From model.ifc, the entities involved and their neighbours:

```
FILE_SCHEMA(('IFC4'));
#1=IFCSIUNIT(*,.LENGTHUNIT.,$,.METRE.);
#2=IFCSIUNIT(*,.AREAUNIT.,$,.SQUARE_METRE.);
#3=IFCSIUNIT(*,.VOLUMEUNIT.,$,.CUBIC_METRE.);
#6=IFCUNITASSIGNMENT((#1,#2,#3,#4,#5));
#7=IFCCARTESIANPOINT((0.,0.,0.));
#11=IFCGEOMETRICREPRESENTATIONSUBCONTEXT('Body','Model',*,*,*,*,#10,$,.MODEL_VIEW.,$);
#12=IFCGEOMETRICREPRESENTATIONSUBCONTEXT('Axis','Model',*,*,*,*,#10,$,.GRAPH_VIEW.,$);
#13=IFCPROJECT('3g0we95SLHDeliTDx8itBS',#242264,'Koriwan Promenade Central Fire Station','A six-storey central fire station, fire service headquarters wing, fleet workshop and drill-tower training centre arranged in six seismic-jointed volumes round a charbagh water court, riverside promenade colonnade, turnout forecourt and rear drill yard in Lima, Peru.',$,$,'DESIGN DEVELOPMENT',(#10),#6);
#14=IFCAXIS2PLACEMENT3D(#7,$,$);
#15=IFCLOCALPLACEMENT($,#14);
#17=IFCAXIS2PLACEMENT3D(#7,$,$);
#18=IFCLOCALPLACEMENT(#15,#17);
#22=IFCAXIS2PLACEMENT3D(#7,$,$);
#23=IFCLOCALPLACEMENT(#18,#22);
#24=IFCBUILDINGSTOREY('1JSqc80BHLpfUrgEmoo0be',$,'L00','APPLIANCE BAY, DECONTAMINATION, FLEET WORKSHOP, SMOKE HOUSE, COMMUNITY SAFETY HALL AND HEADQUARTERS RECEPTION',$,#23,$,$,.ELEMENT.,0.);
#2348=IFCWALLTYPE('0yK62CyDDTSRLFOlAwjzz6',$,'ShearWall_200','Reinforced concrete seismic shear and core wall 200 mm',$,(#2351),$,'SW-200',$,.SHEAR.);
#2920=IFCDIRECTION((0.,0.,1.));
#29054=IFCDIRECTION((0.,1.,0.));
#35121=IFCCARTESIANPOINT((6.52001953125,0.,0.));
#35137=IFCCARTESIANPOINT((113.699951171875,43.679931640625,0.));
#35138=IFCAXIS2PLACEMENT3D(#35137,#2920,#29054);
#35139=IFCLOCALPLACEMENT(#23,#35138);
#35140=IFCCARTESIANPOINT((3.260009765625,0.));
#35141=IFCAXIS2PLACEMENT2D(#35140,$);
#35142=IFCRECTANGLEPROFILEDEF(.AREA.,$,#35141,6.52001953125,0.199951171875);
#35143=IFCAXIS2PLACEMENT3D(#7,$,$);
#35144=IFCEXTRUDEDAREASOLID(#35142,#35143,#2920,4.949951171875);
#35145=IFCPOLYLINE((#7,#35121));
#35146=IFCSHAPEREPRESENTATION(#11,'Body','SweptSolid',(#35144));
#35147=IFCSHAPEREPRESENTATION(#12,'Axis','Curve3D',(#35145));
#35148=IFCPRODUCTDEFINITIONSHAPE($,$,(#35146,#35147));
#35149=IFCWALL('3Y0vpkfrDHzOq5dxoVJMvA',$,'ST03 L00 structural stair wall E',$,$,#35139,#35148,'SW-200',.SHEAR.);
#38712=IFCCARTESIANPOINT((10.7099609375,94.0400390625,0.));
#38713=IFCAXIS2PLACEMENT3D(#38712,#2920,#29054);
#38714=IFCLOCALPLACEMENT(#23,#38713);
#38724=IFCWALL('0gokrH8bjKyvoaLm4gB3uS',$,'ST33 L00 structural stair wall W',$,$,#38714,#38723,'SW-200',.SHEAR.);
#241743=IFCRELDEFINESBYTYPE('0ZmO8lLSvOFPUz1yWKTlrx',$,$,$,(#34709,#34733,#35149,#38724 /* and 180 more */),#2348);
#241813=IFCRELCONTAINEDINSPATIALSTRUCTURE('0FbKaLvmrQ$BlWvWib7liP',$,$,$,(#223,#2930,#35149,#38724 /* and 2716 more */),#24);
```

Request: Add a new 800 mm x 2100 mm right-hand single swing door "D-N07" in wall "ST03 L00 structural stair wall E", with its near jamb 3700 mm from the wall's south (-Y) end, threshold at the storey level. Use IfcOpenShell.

```python
import numpy as np
import ifcopenshell
import ifcopenshell.api.feature
import ifcopenshell.api.geometry
import ifcopenshell.api.root
import ifcopenshell.api.spatial
import ifcopenshell.geom
import ifcopenshell.util.element
import ifcopenshell.util.placement
import ifcopenshell.util.representation
import ifcopenshell.util.shape
import ifcopenshell.util.unit

model = ifcopenshell.open("model.ifc")
unit_scale = ifcopenshell.util.unit.calculate_unit_scale(model)
settings = ifcopenshell.geom.settings()


def volume(element):
    """Net volume in cubic metres, openings subtracted."""
    shape = ifcopenshell.geom.create_shape(settings, element)
    return ifcopenshell.util.shape.get_volume(shape.geometry)


wall = model.by_guid("3Y0vpkfrDHzOq5dxoVJMvA")
storey = ifcopenshell.util.element.get_container(wall, ifc_class="IfcBuildingStorey")
context = ifcopenshell.util.representation.get_context(model, "Model", "Body", "MODEL_VIEW")
before = volume(wall)

width, height, from_end, sill = 0.8, 2.1, 3.7, 0.0  # metres

# The wall runs along its own X axis, and the end named is its -X end.
wall_shape = ifcopenshell.geom.create_shape(settings, wall)
x, y, z = ifcopenshell.util.shape.get_vertices(wall_shape.geometry).T
start = x.min() + from_end
face, thickness = float(y.min()), float(y.max() - y.min())
wall_matrix = ifcopenshell.util.placement.get_local_placement(wall.ObjectPlacement)
level = ifcopenshell.util.placement.get_local_placement(storey.ObjectPlacement)[2, 3]


def in_wall(x, y):
    """Placement at x, y metres in the wall's axes, at sill height."""
    matrix = wall_matrix.copy()
    matrix[:, 3] = wall_matrix @ np.array([x / unit_scale, y / unit_scale, 0.0, 1.0])
    matrix[2, 3] = level + sill / unit_scale
    return matrix


# Opening: a box that overshoots both wall faces by 50 mm.
opening = ifcopenshell.api.root.create_entity(model, ifc_class="IfcOpeningElement", predefined_type="OPENING")
box = ifcopenshell.api.geometry.add_wall_representation(
    model, context=context, length=width, height=height, thickness=thickness + 0.1
)
ifcopenshell.api.geometry.assign_representation(model, product=opening, representation=box)
ifcopenshell.api.geometry.edit_object_placement(model, product=opening, matrix=in_wall(start, face - 0.05), is_si=False)
ifcopenshell.api.feature.add_feature(model, feature=opening, element=wall)

door = ifcopenshell.api.root.create_entity(model, ifc_class="IfcDoor", name="D-N07", predefined_type="DOOR")
door.OverallWidth, door.OverallHeight = width / unit_scale, height / unit_scale
door.OperationType = "SINGLE_SWING_RIGHT"
body = ifcopenshell.api.geometry.add_door_representation(
    model,
    context=context,
    overall_width=door.OverallWidth,
    overall_height=door.OverallHeight,
    operation_type="SINGLE_SWING_RIGHT",
    lining_properties={"LiningDepth": thickness / unit_scale, "ThresholdDepth": thickness / unit_scale},
)
ifcopenshell.api.geometry.assign_representation(model, product=door, representation=body)
ifcopenshell.api.spatial.assign_container(model, products=[door], relating_structure=storey)
ifcopenshell.api.feature.add_filling(model, opening=opening, element=door)

# The lining spans the wall, so the door starts at the wall face.
ifcopenshell.api.geometry.edit_object_placement(model, product=door, matrix=in_wall(start, face), is_si=False)

after = volume(wall)

print(f"wall volume {before:.3f} -> {after:.3f} m3")

model.write("model_edited.ifc")
```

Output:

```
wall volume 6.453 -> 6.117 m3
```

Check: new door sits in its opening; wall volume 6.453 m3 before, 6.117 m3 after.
